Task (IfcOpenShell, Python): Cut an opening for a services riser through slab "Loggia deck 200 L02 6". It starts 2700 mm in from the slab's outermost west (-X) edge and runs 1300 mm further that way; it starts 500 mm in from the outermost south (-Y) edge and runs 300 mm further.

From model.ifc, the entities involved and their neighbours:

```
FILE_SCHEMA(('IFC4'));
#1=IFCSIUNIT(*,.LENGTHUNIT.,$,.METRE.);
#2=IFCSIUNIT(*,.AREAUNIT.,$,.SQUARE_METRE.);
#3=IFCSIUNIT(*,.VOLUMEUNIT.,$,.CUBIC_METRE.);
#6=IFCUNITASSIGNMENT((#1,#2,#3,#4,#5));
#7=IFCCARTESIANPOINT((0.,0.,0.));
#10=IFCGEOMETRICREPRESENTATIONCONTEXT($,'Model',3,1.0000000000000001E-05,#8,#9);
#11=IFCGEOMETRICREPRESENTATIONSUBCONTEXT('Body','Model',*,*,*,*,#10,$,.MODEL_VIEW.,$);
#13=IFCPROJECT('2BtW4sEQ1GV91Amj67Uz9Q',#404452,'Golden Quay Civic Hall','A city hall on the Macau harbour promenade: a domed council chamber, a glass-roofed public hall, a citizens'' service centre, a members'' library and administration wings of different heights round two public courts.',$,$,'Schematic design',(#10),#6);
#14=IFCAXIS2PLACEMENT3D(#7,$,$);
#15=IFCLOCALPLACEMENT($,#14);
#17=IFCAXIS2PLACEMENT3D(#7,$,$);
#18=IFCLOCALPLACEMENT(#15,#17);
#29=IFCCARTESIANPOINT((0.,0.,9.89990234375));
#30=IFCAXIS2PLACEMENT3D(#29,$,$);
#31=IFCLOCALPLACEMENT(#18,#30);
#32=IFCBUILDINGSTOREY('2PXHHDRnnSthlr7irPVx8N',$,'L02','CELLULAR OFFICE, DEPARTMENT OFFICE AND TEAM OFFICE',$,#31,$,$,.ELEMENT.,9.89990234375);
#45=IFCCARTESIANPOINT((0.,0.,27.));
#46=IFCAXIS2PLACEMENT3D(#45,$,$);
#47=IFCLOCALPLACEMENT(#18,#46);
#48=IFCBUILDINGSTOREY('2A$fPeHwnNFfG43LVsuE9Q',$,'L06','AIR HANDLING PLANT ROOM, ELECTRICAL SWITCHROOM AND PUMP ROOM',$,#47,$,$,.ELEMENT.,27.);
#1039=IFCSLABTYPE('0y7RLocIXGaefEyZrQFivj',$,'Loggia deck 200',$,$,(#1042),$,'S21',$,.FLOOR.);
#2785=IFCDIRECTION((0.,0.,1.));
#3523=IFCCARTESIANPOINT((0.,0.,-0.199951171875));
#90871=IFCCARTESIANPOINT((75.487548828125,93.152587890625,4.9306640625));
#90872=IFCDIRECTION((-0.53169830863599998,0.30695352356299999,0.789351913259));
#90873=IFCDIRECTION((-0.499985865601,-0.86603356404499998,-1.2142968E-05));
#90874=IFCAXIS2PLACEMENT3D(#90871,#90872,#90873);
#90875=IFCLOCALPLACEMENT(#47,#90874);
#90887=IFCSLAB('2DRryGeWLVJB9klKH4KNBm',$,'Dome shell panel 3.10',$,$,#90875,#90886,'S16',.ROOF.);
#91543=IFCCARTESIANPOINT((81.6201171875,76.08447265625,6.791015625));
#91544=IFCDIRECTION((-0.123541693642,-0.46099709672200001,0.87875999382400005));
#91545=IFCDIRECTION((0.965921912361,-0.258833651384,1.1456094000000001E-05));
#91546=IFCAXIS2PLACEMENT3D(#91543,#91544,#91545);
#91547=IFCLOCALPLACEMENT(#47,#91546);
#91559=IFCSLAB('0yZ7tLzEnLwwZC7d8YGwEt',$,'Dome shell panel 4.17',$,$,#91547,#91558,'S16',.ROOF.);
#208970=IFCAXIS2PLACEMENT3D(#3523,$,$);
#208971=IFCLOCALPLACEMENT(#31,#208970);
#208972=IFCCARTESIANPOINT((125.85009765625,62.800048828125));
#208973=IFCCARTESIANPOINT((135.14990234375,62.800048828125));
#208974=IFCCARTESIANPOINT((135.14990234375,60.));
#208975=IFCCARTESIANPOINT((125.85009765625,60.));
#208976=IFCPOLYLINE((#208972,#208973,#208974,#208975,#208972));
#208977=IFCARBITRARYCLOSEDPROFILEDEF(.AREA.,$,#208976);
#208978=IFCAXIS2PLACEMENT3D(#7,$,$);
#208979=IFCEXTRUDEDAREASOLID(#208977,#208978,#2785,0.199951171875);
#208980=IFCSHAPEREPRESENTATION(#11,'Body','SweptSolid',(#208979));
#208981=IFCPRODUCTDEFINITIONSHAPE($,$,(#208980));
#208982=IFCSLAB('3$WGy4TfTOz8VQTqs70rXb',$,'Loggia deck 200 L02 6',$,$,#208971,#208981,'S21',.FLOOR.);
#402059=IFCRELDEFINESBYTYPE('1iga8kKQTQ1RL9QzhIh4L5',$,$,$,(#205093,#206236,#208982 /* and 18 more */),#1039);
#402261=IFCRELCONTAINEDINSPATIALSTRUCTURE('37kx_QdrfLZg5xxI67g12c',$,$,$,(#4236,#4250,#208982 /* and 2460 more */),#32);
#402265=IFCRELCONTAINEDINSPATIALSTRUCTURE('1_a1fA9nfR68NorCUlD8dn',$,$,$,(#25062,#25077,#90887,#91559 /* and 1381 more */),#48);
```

```python
import numpy as np
import ifcopenshell
import ifcopenshell.api.feature
import ifcopenshell.api.geometry
import ifcopenshell.api.root
import ifcopenshell.geom
import ifcopenshell.util.placement
import ifcopenshell.util.representation
import ifcopenshell.util.shape
import ifcopenshell.util.unit

model = ifcopenshell.open("model.ifc")
unit_scale = ifcopenshell.util.unit.calculate_unit_scale(model)
settings = ifcopenshell.geom.settings()


def volume(element):
    """Net volume in cubic metres, openings subtracted."""
    shape = ifcopenshell.geom.create_shape(settings, element)
    return ifcopenshell.util.shape.get_volume(shape.geometry)


slab = model.by_guid("3$WGy4TfTOz8VQTqs70rXb")
before = volume(slab)

# Extent in the slab's own axes, in metres. The edges named are its -X and -Y sides.
slab_shape = ifcopenshell.geom.create_shape(settings, slab)
vertices = ifcopenshell.util.shape.get_vertices(slab_shape.geometry)
x_min, y_min, bottom = vertices.min(axis=0)
top = vertices[:, 2].max()

opening = ifcopenshell.api.root.create_entity(model, ifc_class="IfcOpeningElement", name="Services riser opening", predefined_type="OPENING")
context = ifcopenshell.util.representation.get_context(model, "Model", "Body", "MODEL_VIEW")
width, depth = 1.3, 0.3
outline = [(0.0, 0.0), (width, 0.0), (width, depth), (0.0, depth), (0.0, 0.0)]
# Overshoot both faces by 50 mm so the cut is clean.
shape = ifcopenshell.api.geometry.add_slab_representation(
    model, context=context, depth=top - bottom + 0.1, polyline=outline
)
ifcopenshell.api.geometry.assign_representation(model, product=opening, representation=shape)

matrix = ifcopenshell.util.placement.get_local_placement(slab.ObjectPlacement)
matrix[:, 3] = matrix @ np.append(np.array([x_min + 2.7, y_min + 0.5, bottom - 0.05]) / unit_scale, 1.0)
ifcopenshell.api.geometry.edit_object_placement(model, product=opening, matrix=matrix, is_si=False)
ifcopenshell.api.feature.add_feature(model, feature=opening, element=slab)

after = volume(slab)

print(f"slab volume {before:.3f} -> {after:.3f} m3")

model.write("model_edited.ifc")
```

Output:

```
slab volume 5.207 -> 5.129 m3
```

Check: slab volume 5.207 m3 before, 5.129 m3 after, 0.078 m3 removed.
